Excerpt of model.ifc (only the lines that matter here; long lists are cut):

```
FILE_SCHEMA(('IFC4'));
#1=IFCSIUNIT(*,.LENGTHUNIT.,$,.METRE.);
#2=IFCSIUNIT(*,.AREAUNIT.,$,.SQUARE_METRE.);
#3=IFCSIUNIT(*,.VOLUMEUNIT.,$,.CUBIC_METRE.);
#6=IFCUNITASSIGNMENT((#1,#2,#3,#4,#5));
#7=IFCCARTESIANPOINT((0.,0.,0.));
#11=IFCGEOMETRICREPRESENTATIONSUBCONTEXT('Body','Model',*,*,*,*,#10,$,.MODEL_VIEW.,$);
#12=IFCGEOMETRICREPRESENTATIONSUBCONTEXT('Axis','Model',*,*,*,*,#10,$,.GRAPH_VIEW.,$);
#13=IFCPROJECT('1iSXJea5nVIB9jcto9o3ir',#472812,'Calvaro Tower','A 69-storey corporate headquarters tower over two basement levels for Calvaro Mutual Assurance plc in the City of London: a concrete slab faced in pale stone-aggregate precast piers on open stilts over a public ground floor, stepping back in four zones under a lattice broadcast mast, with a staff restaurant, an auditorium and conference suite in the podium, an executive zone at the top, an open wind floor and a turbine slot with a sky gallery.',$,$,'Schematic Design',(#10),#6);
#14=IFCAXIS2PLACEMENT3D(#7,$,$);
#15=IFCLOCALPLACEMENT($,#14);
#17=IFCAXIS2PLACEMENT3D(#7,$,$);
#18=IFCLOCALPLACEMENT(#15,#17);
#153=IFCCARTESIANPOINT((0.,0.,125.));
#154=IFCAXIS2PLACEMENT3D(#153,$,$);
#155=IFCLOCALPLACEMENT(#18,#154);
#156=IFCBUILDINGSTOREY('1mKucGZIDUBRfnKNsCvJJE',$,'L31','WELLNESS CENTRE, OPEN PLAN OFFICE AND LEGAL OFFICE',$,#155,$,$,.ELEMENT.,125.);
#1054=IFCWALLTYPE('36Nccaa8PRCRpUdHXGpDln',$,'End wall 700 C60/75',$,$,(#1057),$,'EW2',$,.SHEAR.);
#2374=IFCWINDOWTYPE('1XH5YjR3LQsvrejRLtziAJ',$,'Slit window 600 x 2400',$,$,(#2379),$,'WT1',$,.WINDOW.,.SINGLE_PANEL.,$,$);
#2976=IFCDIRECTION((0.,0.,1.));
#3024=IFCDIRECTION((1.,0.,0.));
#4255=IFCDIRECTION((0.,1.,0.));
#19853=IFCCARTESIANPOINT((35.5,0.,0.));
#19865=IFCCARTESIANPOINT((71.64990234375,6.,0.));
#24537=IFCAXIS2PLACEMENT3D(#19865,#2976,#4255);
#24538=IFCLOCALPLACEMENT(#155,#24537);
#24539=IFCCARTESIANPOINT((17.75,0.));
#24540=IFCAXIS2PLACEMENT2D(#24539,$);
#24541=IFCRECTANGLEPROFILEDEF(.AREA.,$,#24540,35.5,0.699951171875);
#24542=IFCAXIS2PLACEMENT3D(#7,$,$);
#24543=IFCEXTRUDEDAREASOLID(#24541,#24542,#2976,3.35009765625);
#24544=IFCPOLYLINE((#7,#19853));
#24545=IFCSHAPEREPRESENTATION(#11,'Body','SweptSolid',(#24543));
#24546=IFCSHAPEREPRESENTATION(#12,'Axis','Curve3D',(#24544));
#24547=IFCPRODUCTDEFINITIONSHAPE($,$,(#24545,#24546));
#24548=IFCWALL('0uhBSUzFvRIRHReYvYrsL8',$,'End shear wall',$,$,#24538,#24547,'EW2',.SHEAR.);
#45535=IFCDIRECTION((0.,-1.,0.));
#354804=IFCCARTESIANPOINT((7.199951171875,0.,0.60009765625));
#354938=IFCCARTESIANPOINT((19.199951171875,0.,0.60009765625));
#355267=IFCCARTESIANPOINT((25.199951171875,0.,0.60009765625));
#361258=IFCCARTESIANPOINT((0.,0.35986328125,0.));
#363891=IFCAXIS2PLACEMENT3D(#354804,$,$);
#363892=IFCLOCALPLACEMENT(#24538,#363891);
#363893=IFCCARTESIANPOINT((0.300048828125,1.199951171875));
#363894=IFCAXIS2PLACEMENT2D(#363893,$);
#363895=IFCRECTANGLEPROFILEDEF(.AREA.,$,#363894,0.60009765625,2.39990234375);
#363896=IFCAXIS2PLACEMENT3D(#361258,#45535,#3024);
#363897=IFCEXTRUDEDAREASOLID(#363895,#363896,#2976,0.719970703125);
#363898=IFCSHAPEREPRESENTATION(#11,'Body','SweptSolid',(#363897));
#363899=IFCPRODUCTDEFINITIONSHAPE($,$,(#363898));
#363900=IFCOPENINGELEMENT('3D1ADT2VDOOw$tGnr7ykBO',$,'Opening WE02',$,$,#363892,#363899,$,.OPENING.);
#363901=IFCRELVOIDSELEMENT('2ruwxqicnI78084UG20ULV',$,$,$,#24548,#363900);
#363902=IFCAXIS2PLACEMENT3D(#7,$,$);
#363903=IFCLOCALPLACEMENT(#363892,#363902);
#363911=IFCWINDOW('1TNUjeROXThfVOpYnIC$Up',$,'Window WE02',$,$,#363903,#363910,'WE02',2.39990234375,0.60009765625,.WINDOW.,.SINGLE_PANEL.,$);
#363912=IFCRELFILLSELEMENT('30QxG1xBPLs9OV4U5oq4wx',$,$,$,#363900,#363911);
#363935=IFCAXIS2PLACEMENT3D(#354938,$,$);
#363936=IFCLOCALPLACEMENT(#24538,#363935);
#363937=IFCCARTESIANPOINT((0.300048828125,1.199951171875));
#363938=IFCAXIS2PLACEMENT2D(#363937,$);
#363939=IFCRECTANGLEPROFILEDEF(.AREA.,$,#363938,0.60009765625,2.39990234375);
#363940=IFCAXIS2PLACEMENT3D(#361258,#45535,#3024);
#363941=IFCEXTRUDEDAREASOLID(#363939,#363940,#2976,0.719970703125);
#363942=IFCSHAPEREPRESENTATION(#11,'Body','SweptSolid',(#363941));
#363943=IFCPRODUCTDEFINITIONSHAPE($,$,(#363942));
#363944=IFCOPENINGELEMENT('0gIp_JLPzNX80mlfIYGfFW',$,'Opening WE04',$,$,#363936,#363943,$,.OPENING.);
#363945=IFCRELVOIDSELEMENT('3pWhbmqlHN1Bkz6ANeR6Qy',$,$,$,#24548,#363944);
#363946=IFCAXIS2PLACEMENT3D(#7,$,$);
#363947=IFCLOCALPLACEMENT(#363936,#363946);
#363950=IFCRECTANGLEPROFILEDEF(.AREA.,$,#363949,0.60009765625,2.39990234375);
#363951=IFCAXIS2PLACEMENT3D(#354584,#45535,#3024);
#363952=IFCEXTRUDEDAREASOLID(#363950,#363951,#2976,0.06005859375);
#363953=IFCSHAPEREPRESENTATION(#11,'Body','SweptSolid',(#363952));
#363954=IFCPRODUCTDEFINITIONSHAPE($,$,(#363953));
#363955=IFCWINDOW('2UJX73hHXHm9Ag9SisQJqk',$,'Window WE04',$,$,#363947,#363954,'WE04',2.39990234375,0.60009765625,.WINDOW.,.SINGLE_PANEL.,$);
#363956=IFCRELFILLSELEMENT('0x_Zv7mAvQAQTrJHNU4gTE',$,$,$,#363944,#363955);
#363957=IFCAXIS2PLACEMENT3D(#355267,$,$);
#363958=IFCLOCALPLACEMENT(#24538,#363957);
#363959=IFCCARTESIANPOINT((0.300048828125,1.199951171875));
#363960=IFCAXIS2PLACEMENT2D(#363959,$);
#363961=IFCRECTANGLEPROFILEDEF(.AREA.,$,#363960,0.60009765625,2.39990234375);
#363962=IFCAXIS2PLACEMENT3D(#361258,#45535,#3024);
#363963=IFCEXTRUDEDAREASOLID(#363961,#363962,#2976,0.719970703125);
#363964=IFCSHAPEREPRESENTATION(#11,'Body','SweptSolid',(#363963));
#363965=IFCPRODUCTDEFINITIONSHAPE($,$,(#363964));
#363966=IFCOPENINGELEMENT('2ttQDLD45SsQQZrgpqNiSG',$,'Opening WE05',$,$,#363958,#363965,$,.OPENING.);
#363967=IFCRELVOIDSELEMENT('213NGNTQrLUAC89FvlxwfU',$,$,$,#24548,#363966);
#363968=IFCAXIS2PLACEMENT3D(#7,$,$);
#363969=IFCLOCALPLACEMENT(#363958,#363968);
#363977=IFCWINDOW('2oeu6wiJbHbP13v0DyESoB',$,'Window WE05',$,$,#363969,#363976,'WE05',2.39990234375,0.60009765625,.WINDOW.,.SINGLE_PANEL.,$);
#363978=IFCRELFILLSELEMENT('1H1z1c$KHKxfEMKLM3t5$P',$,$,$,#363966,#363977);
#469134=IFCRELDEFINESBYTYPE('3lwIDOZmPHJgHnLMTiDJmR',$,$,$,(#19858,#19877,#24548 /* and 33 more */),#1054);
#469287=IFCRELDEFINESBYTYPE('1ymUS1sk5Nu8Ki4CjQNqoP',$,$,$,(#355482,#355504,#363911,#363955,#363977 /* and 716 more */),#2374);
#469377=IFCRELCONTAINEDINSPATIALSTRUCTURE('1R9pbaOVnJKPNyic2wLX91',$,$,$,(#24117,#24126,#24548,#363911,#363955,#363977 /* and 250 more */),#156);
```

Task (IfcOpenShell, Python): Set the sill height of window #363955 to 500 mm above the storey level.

```python
import numpy as np
import ifcopenshell
import ifcopenshell.api.geometry
import ifcopenshell.geom
import ifcopenshell.util.element
import ifcopenshell.util.placement
import ifcopenshell.util.shape
import ifcopenshell.util.unit

model = ifcopenshell.open("model.ifc")
unit_scale = ifcopenshell.util.unit.calculate_unit_scale(model)

window = model.by_guid("2UJX73hHXHm9Ag9SisQJqk")
opening = window.FillsVoids[0].RelatingOpeningElement
storey = ifcopenshell.util.element.get_container(window, ifc_class="IfcBuildingStorey")
level = ifcopenshell.util.placement.get_local_placement(storey.ObjectPlacement)[2, 3]

# The opening's origin need not be at the sill, so measure its lowest point.
shape = ifcopenshell.geom.create_shape(ifcopenshell.geom.settings(), opening)
bottom = ifcopenshell.util.shape.get_shape_bottom_elevation(shape, shape.geometry) / unit_scale
dz = level + 0.5 / unit_scale - bottom

shift = np.array([0.0, 0.0, dz])
# The window is placed relative to its opening, so it follows when the opening moves.
matrix = ifcopenshell.util.placement.get_local_placement(opening.ObjectPlacement)
matrix[:3, 3] += shift
ifcopenshell.api.geometry.edit_object_placement(
    model, product=opening, matrix=matrix, is_si=False, should_transform_children=True
)

print(f"moved by {dz * unit_scale:+.3f} m")

model.write("model_v2.ifc")
```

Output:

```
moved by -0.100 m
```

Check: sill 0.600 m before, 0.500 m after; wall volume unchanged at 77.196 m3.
